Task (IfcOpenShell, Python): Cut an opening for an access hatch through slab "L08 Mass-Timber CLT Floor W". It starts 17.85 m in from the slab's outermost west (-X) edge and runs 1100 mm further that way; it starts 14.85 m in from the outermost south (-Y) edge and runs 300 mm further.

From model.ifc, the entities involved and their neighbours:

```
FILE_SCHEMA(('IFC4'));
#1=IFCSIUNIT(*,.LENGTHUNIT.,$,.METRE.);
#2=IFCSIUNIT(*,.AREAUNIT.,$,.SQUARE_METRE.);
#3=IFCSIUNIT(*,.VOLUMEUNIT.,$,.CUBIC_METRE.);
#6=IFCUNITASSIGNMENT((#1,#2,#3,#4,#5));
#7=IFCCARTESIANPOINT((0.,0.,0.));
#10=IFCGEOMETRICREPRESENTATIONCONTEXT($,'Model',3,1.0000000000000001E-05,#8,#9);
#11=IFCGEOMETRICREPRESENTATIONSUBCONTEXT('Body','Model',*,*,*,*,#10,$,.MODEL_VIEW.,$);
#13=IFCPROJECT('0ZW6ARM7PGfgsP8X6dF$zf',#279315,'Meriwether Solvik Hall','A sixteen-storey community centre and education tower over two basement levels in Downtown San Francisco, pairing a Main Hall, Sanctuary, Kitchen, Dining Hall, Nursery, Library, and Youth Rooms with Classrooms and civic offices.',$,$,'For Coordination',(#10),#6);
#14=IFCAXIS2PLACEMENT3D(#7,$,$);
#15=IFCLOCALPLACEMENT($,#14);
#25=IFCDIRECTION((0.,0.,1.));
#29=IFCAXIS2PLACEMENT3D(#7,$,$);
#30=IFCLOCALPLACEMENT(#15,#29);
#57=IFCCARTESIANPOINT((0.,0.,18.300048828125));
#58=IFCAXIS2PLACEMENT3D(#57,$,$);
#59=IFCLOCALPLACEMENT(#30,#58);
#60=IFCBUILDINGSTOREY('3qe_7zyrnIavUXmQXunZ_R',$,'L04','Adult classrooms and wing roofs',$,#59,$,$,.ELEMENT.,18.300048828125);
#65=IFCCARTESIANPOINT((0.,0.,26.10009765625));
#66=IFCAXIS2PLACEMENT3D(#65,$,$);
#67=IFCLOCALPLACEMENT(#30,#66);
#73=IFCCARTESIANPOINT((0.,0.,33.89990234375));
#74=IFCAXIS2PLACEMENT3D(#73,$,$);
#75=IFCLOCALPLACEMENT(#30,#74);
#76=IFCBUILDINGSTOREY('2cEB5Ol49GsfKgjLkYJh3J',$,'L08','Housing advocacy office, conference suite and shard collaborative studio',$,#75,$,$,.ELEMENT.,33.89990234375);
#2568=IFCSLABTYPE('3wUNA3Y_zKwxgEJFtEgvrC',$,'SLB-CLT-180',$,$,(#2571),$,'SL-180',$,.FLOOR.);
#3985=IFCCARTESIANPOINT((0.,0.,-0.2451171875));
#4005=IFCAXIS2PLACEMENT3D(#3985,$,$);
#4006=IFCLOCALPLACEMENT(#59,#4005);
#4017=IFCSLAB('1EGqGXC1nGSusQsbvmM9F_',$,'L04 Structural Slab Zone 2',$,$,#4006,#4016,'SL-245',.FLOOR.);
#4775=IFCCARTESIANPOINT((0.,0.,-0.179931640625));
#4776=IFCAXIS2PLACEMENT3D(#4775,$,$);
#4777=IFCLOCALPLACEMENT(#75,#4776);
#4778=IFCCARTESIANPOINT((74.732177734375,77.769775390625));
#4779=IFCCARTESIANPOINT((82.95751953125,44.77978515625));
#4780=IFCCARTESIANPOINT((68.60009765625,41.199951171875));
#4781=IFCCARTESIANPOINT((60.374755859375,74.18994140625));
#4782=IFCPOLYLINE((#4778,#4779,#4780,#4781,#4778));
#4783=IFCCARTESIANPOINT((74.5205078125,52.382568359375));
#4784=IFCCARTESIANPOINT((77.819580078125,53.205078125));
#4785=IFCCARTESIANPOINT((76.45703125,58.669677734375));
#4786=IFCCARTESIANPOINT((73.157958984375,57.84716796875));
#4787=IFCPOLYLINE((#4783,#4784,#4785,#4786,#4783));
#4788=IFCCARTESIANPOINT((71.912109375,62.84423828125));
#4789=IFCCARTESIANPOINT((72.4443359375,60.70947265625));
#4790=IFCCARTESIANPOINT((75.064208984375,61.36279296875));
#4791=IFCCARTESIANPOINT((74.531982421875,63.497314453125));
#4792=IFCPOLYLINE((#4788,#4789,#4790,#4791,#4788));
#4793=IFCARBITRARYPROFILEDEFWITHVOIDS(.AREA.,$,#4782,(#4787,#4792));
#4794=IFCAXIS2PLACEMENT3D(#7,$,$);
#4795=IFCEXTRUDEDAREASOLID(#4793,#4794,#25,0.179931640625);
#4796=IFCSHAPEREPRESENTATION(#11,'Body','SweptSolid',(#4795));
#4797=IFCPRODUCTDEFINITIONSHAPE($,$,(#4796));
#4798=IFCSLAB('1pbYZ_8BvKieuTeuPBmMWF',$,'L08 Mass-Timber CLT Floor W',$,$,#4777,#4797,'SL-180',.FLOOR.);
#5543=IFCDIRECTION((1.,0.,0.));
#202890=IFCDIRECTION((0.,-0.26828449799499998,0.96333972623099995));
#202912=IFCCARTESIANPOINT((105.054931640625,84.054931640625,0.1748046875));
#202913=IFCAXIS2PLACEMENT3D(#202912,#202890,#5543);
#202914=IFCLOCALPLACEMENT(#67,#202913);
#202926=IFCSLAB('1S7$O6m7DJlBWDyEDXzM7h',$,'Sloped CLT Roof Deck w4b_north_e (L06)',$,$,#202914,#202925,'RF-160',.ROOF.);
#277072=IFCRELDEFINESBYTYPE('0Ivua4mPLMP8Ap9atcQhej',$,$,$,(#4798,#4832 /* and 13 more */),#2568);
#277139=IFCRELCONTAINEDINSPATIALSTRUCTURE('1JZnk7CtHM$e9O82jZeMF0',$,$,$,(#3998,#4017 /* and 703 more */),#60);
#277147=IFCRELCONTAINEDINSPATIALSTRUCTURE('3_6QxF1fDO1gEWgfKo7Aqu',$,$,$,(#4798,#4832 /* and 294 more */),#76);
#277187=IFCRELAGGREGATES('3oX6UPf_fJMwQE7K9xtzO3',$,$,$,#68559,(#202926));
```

```python
import numpy as np
import ifcopenshell
import ifcopenshell.api.feature
import ifcopenshell.api.geometry
import ifcopenshell.api.root
import ifcopenshell.geom
import ifcopenshell.util.placement
import ifcopenshell.util.representation
import ifcopenshell.util.shape
import ifcopenshell.util.unit

model = ifcopenshell.open("model.ifc")
unit_scale = ifcopenshell.util.unit.calculate_unit_scale(model)
settings = ifcopenshell.geom.settings()


def volume(element):
    """Net volume in cubic metres, openings subtracted."""
    shape = ifcopenshell.geom.create_shape(settings, element)
    return ifcopenshell.util.shape.get_volume(shape.geometry)


slab = model.by_guid("1pbYZ_8BvKieuTeuPBmMWF")
before = volume(slab)

# Extent in the slab's own axes, in metres. The edges named are its -X and -Y sides.
slab_shape = ifcopenshell.geom.create_shape(settings, slab)
vertices = ifcopenshell.util.shape.get_vertices(slab_shape.geometry)
x_min, y_min, bottom = vertices.min(axis=0)
top = vertices[:, 2].max()

opening = ifcopenshell.api.root.create_entity(model, ifc_class="IfcOpeningElement", name="Access hatch opening", predefined_type="OPENING")
context = ifcopenshell.util.representation.get_context(model, "Model", "Body", "MODEL_VIEW")
width, depth = 1.1, 0.3
outline = [(0.0, 0.0), (width, 0.0), (width, depth), (0.0, depth), (0.0, 0.0)]
# Overshoot both faces by 50 mm so the cut is clean.
shape = ifcopenshell.api.geometry.add_slab_representation(
    model, context=context, depth=top - bottom + 0.1, polyline=outline
)
ifcopenshell.api.geometry.assign_representation(model, product=opening, representation=shape)

matrix = ifcopenshell.util.placement.get_local_placement(slab.ObjectPlacement)
matrix[:, 3] = matrix @ np.append(np.array([x_min + 17.85, y_min + 14.85, bottom - 0.05]) / unit_scale, 1.0)
ifcopenshell.api.geometry.edit_object_placement(model, product=opening, matrix=matrix, is_si=False)
ifcopenshell.api.feature.add_feature(model, feature=opening, element=slab)

after = volume(slab)

print(f"slab volume {before:.3f} -> {after:.3f} m3")

model.write("model_edited.ifc")
```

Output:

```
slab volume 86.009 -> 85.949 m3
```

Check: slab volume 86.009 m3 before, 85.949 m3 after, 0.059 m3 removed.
